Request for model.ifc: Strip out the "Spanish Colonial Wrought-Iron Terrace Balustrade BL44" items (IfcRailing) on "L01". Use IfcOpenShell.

First a look at what the model holds.

```python
import ifcopenshell
import ifcopenshell.util.element

model = ifcopenshell.open("model.ifc")
print(model.schema)
storey = next(s for s in model.by_type("IfcBuildingStorey") if s.Name == "L01")
railings = [e for e in ifcopenshell.util.element.get_decomposition(storey) if e.is_a("IfcRailing")]
seen = {}
for e in railings:
    element_type = ifcopenshell.util.element.get_type(e)
    name = element_type.Name if element_type not in (None, e) else None
    seen[name] = seen.get(name, 0) + 1
for name, count in sorted(seen.items(), key=str):
    print(count, "x", name)
```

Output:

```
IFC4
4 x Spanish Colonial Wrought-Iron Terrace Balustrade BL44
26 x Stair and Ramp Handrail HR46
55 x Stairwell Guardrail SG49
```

```python
import ifcopenshell
import ifcopenshell.api.root
import ifcopenshell.util.element

model = ifcopenshell.open("model.ifc")

storey = next(s for s in model.by_type("IfcBuildingStorey") if s.Name == "L01")
railings = [e for e in ifcopenshell.util.element.get_decomposition(storey) if e.is_a("IfcRailing")]
targets = [e for e in railings if (t := ifcopenshell.util.element.get_type(e)) not in (None, e) and t.Name == "Spanish Colonial Wrought-Iron Terrace Balustrade BL44"]

for e in targets:
    ifcopenshell.api.root.remove_product(model, product=e)
print(len(targets), "removed")

model.write("model_v2.ifc")
```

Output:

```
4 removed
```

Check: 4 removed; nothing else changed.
